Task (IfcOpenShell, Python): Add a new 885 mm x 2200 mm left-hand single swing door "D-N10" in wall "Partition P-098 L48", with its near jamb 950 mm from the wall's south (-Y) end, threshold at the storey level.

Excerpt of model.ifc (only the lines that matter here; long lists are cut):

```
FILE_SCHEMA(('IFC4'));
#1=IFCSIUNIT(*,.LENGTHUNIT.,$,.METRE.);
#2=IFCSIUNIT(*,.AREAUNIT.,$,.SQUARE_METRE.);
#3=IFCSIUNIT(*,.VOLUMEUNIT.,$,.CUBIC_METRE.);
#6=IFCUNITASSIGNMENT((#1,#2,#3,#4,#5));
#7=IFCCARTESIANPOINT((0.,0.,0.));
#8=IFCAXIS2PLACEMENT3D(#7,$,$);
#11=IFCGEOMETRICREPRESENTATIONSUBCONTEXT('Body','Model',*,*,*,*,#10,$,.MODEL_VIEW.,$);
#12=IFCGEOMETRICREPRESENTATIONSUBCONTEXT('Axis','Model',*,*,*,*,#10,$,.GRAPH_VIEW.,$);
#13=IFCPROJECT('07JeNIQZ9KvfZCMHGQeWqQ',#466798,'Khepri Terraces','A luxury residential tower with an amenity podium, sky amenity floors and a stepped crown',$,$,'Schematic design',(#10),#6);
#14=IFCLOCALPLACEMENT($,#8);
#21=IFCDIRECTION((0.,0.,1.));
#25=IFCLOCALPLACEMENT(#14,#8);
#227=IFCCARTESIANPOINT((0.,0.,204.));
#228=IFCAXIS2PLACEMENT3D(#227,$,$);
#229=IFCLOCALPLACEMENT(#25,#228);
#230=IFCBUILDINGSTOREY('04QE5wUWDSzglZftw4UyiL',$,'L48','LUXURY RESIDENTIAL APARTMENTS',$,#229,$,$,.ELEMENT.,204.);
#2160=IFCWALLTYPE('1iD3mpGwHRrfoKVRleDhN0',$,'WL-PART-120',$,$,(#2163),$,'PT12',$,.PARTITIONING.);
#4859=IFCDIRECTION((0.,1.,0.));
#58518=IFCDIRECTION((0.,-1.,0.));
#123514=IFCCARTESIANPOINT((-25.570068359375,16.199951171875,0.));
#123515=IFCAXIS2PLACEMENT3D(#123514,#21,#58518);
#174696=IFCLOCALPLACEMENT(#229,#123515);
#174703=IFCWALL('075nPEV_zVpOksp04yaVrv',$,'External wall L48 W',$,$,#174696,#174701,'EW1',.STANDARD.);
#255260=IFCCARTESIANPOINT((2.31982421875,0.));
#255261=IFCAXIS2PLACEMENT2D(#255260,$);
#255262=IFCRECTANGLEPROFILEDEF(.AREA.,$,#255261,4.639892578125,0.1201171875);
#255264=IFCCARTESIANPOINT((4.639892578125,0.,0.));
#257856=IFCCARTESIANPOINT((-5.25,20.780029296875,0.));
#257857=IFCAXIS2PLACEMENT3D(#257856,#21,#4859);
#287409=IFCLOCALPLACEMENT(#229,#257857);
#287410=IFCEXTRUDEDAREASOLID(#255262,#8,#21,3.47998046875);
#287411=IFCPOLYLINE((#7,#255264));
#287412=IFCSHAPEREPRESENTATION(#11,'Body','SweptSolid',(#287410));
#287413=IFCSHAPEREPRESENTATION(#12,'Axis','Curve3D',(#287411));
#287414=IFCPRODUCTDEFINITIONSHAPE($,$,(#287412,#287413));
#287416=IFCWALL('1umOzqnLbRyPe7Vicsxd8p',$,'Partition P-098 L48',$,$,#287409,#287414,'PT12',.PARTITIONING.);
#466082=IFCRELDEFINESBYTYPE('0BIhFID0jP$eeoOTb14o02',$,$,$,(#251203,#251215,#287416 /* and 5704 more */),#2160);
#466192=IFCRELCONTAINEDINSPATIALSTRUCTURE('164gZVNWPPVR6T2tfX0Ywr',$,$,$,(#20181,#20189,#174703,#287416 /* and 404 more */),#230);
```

```python
import numpy as np
import ifcopenshell
import ifcopenshell.api.feature
import ifcopenshell.api.geometry
import ifcopenshell.api.root
import ifcopenshell.api.spatial
import ifcopenshell.geom
import ifcopenshell.util.element
import ifcopenshell.util.placement
import ifcopenshell.util.representation
import ifcopenshell.util.shape
import ifcopenshell.util.unit

model = ifcopenshell.open("model.ifc")
unit_scale = ifcopenshell.util.unit.calculate_unit_scale(model)
settings = ifcopenshell.geom.settings()


def volume(element):
    """Net volume in cubic metres, openings subtracted."""
    shape = ifcopenshell.geom.create_shape(settings, element)
    return ifcopenshell.util.shape.get_volume(shape.geometry)


wall = model.by_guid("1umOzqnLbRyPe7Vicsxd8p")
storey = ifcopenshell.util.element.get_container(wall, ifc_class="IfcBuildingStorey")
context = ifcopenshell.util.representation.get_context(model, "Model", "Body", "MODEL_VIEW")
before = volume(wall)

width, height, from_end, sill = 0.885, 2.2, 0.95, 0.0  # metres

# The wall runs along its own X axis, and the end named is its -X end.
wall_shape = ifcopenshell.geom.create_shape(settings, wall)
x, y, z = ifcopenshell.util.shape.get_vertices(wall_shape.geometry).T
start = x.min() + from_end
face, thickness = float(y.min()), float(y.max() - y.min())
wall_matrix = ifcopenshell.util.placement.get_local_placement(wall.ObjectPlacement)
level = ifcopenshell.util.placement.get_local_placement(storey.ObjectPlacement)[2, 3]


def in_wall(x, y):
    """Placement at x, y metres in the wall's axes, at sill height."""
    matrix = wall_matrix.copy()
    matrix[:, 3] = wall_matrix @ np.array([x / unit_scale, y / unit_scale, 0.0, 1.0])
    matrix[2, 3] = level + sill / unit_scale
    return matrix


# Opening: a box that overshoots both wall faces by 50 mm.
opening = ifcopenshell.api.root.create_entity(model, ifc_class="IfcOpeningElement", predefined_type="OPENING")
box = ifcopenshell.api.geometry.add_wall_representation(
    model, context=context, length=width, height=height, thickness=thickness + 0.1
)
ifcopenshell.api.geometry.assign_representation(model, product=opening, representation=box)
ifcopenshell.api.geometry.edit_object_placement(model, product=opening, matrix=in_wall(start, face - 0.05), is_si=False)
ifcopenshell.api.feature.add_feature(model, feature=opening, element=wall)

door = ifcopenshell.api.root.create_entity(model, ifc_class="IfcDoor", name="D-N10", predefined_type="DOOR")
door.OverallWidth, door.OverallHeight = width / unit_scale, height / unit_scale
door.OperationType = "SINGLE_SWING_LEFT"
body = ifcopenshell.api.geometry.add_door_representation(
    model,
    context=context,
    overall_width=door.OverallWidth,
    overall_height=door.OverallHeight,
    operation_type="SINGLE_SWING_LEFT",
    lining_properties={"LiningDepth": thickness / unit_scale, "ThresholdDepth": thickness / unit_scale},
)
ifcopenshell.api.geometry.assign_representation(model, product=door, representation=body)
ifcopenshell.api.spatial.assign_container(model, products=[door], relating_structure=storey)
ifcopenshell.api.feature.add_filling(model, opening=opening, element=door)

# The lining spans the wall, so the door starts at the wall face.
ifcopenshell.api.geometry.edit_object_placement(model, product=door, matrix=in_wall(start, face), is_si=False)

after = volume(wall)

print(f"wall volume {before:.3f} -> {after:.3f} m3")

model.write("model_edited.ifc")
```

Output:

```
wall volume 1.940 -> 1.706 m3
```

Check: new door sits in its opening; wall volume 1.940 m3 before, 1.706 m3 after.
